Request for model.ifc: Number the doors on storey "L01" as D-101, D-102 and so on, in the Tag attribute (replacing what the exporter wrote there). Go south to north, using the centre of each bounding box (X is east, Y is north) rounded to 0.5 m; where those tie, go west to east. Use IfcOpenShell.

First a look at what the model holds.

```python
import ifcopenshell
import ifcopenshell.util.element
import ifcopenshell.util.placement

model = ifcopenshell.open("model.ifc")
print(model.schema)
storey = next(s for s in model.by_type("IfcBuildingStorey") if s.Name == "L01")
doors = [e for e in ifcopenshell.util.element.get_decomposition(storey) if e.is_a("IfcDoor")]
for e in sorted(doors, key=lambda e: e.id()):
    origin = ifcopenshell.util.placement.get_local_placement(e.ObjectPlacement)[:3, 3]
    print(e.id(), e.Tag, e.Name, origin.round(2) + 0.0, sep=" | ")
```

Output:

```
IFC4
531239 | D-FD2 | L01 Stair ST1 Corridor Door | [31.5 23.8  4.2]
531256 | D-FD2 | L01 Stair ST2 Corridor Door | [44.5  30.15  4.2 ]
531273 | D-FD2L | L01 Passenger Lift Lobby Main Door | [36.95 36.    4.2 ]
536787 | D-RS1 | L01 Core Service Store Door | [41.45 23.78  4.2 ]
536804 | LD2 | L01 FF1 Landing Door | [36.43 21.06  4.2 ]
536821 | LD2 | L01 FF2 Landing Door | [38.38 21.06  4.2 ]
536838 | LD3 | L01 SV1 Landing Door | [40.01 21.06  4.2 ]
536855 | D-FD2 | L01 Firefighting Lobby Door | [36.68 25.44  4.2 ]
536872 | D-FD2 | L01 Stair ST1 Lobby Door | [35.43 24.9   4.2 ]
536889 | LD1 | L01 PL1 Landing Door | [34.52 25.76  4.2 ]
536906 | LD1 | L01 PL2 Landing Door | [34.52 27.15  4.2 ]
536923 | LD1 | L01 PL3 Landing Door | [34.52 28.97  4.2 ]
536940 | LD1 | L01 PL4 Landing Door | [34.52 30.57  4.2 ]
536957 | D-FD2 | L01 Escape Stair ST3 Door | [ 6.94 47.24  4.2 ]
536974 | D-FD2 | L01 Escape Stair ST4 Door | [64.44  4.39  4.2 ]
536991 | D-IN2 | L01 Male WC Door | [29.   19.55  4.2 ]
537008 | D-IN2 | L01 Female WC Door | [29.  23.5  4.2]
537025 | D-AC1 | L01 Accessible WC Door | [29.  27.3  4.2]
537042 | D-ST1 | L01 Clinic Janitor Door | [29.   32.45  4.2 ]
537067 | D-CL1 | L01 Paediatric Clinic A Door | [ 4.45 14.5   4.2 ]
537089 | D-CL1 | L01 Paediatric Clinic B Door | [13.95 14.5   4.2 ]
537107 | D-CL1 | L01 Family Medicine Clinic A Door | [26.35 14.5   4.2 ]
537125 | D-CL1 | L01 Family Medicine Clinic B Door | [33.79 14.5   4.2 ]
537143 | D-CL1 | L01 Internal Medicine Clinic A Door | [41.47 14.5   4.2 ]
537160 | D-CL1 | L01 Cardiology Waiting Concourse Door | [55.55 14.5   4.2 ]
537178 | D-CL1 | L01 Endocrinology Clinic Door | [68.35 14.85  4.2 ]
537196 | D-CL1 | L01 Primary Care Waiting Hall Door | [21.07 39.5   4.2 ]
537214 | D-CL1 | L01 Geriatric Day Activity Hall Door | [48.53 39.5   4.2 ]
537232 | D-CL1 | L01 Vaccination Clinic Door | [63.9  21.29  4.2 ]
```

```python
import ifcopenshell
import ifcopenshell.geom
import ifcopenshell.util.element
import ifcopenshell.util.shape

model = ifcopenshell.open("model.ifc")
settings = ifcopenshell.geom.settings()
settings.set("use-world-coords", True)


def centre(element):
    shape = ifcopenshell.geom.create_shape(settings, element)
    return ifcopenshell.util.shape.get_bbox_centroid(shape.geometry)


storey = next(s for s in model.by_type("IfcBuildingStorey") if s.Name == "L01")
doors = [e for e in ifcopenshell.util.element.get_decomposition(storey) if e.is_a("IfcDoor")]

# Insertion points can sit at a corner or the storey origin, so sort by the geometry (in metres).
centres = {e: centre(e) for e in doors}
doors.sort(key=lambda e: (round(centres[e][1] / 0.5), centres[e][0]))

for i, e in enumerate(doors, start=1):
    number = f"D-1{i:02d}"
    e.Tag = number
    print(e.id(), number)

model.write("model_updated.ifc")
```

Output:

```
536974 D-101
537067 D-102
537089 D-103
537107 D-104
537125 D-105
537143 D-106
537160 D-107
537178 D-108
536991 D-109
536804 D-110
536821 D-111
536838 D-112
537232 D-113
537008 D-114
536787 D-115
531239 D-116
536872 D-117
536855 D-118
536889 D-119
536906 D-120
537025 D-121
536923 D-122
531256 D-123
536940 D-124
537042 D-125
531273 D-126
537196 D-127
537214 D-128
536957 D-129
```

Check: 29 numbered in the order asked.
